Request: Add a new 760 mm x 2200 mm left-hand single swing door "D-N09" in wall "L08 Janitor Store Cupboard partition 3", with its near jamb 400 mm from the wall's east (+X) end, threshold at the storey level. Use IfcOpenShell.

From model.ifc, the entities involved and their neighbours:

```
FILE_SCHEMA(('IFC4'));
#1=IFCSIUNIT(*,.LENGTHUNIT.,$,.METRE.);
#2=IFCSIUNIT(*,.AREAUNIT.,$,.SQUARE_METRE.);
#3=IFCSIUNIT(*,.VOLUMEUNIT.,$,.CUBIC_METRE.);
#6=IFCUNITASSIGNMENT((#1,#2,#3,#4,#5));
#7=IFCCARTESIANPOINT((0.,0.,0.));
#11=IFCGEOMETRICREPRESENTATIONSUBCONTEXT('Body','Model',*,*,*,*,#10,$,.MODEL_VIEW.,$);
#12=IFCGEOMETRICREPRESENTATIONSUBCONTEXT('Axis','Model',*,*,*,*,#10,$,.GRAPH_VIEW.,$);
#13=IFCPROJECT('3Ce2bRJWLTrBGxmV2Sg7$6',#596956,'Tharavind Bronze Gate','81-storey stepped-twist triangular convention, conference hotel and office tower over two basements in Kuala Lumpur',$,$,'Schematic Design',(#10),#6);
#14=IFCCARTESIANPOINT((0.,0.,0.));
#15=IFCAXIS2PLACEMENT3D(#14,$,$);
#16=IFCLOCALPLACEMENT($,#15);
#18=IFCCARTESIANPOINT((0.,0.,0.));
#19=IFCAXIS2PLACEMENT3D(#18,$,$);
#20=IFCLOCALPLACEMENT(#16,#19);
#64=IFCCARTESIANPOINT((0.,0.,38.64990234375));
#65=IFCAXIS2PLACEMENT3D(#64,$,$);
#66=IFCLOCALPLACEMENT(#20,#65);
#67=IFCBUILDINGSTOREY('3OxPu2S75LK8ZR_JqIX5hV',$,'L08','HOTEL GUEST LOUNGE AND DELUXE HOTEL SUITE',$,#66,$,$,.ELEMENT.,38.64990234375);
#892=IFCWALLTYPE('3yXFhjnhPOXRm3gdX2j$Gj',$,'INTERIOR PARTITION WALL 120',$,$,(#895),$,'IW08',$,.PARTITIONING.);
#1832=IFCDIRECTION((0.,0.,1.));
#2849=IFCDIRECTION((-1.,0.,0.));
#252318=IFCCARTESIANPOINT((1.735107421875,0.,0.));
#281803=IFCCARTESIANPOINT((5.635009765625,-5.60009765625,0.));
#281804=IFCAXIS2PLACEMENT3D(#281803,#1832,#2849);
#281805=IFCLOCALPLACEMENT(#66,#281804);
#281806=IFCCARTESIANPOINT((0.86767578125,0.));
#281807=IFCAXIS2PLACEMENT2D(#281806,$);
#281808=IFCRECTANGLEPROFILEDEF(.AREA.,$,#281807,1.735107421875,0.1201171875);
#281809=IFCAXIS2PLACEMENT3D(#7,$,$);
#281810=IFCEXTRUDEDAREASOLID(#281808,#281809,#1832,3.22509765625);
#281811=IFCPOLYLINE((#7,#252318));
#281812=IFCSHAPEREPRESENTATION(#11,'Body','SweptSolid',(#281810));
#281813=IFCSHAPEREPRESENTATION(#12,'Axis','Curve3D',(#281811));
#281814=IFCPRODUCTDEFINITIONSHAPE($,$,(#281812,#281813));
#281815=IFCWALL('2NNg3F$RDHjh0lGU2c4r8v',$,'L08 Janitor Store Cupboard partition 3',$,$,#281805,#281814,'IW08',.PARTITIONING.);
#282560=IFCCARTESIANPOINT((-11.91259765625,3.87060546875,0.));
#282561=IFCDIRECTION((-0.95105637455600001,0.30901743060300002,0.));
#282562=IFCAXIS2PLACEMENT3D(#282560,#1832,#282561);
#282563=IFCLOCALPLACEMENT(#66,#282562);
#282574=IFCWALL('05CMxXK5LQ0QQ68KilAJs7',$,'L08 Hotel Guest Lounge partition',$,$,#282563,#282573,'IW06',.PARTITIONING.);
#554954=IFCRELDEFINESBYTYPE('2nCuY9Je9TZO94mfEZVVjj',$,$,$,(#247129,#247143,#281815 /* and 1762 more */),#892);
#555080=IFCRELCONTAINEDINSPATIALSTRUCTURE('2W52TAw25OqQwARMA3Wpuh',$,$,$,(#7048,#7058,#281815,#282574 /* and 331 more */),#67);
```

```python
import numpy as np
import ifcopenshell
import ifcopenshell.api.feature
import ifcopenshell.api.geometry
import ifcopenshell.api.root
import ifcopenshell.api.spatial
import ifcopenshell.geom
import ifcopenshell.util.element
import ifcopenshell.util.placement
import ifcopenshell.util.representation
import ifcopenshell.util.shape
import ifcopenshell.util.unit

model = ifcopenshell.open("model.ifc")
unit_scale = ifcopenshell.util.unit.calculate_unit_scale(model)
settings = ifcopenshell.geom.settings()


def volume(element):
    """Net volume in cubic metres, openings subtracted."""
    shape = ifcopenshell.geom.create_shape(settings, element)
    return ifcopenshell.util.shape.get_volume(shape.geometry)


wall = model.by_id(281815)
storey = ifcopenshell.util.element.get_container(wall, ifc_class="IfcBuildingStorey")
context = ifcopenshell.util.representation.get_context(model, "Model", "Body", "MODEL_VIEW")
before = volume(wall)

width, height, from_end, sill = 0.76, 2.2, 0.4, 0.0  # metres

# The wall runs along its own X axis, and the end named is its -X end.
wall_shape = ifcopenshell.geom.create_shape(settings, wall)
x, y, z = ifcopenshell.util.shape.get_vertices(wall_shape.geometry).T
start = x.min() + from_end
face, thickness = float(y.min()), float(y.max() - y.min())
wall_matrix = ifcopenshell.util.placement.get_local_placement(wall.ObjectPlacement)
level = ifcopenshell.util.placement.get_local_placement(storey.ObjectPlacement)[2, 3]


def in_wall(x, y):
    """Placement at x, y metres in the wall's axes, at sill height."""
    matrix = wall_matrix.copy()
    matrix[:, 3] = wall_matrix @ np.array([x / unit_scale, y / unit_scale, 0.0, 1.0])
    matrix[2, 3] = level + sill / unit_scale
    return matrix


# Opening: a box that overshoots both wall faces by 50 mm.
opening = ifcopenshell.api.root.create_entity(model, ifc_class="IfcOpeningElement", predefined_type="OPENING")
box = ifcopenshell.api.geometry.add_wall_representation(
    model, context=context, length=width, height=height, thickness=thickness + 0.1
)
ifcopenshell.api.geometry.assign_representation(model, product=opening, representation=box)
ifcopenshell.api.geometry.edit_object_placement(model, product=opening, matrix=in_wall(start, face - 0.05), is_si=False)
ifcopenshell.api.feature.add_feature(model, feature=opening, element=wall)

door = ifcopenshell.api.root.create_entity(model, ifc_class="IfcDoor", name="D-N09", predefined_type="DOOR")
door.OverallWidth, door.OverallHeight = width / unit_scale, height / unit_scale
door.OperationType = "SINGLE_SWING_LEFT"
body = ifcopenshell.api.geometry.add_door_representation(
    model,
    context=context,
    overall_width=door.OverallWidth,
    overall_height=door.OverallHeight,
    operation_type="SINGLE_SWING_LEFT",
    lining_properties={"LiningDepth": thickness / unit_scale, "ThresholdDepth": thickness / unit_scale},
)
ifcopenshell.api.geometry.assign_representation(model, product=door, representation=body)
ifcopenshell.api.spatial.assign_container(model, products=[door], relating_structure=storey)
ifcopenshell.api.feature.add_filling(model, opening=opening, element=door)

# The lining spans the wall, so the door starts at the wall face.
ifcopenshell.api.geometry.edit_object_placement(model, product=door, matrix=in_wall(start, face), is_si=False)

after = volume(wall)

print(f"wall volume {before:.3f} -> {after:.3f} m3")

model.write("model_v2.ifc")
```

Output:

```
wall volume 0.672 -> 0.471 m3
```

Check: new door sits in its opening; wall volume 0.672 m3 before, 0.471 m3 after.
